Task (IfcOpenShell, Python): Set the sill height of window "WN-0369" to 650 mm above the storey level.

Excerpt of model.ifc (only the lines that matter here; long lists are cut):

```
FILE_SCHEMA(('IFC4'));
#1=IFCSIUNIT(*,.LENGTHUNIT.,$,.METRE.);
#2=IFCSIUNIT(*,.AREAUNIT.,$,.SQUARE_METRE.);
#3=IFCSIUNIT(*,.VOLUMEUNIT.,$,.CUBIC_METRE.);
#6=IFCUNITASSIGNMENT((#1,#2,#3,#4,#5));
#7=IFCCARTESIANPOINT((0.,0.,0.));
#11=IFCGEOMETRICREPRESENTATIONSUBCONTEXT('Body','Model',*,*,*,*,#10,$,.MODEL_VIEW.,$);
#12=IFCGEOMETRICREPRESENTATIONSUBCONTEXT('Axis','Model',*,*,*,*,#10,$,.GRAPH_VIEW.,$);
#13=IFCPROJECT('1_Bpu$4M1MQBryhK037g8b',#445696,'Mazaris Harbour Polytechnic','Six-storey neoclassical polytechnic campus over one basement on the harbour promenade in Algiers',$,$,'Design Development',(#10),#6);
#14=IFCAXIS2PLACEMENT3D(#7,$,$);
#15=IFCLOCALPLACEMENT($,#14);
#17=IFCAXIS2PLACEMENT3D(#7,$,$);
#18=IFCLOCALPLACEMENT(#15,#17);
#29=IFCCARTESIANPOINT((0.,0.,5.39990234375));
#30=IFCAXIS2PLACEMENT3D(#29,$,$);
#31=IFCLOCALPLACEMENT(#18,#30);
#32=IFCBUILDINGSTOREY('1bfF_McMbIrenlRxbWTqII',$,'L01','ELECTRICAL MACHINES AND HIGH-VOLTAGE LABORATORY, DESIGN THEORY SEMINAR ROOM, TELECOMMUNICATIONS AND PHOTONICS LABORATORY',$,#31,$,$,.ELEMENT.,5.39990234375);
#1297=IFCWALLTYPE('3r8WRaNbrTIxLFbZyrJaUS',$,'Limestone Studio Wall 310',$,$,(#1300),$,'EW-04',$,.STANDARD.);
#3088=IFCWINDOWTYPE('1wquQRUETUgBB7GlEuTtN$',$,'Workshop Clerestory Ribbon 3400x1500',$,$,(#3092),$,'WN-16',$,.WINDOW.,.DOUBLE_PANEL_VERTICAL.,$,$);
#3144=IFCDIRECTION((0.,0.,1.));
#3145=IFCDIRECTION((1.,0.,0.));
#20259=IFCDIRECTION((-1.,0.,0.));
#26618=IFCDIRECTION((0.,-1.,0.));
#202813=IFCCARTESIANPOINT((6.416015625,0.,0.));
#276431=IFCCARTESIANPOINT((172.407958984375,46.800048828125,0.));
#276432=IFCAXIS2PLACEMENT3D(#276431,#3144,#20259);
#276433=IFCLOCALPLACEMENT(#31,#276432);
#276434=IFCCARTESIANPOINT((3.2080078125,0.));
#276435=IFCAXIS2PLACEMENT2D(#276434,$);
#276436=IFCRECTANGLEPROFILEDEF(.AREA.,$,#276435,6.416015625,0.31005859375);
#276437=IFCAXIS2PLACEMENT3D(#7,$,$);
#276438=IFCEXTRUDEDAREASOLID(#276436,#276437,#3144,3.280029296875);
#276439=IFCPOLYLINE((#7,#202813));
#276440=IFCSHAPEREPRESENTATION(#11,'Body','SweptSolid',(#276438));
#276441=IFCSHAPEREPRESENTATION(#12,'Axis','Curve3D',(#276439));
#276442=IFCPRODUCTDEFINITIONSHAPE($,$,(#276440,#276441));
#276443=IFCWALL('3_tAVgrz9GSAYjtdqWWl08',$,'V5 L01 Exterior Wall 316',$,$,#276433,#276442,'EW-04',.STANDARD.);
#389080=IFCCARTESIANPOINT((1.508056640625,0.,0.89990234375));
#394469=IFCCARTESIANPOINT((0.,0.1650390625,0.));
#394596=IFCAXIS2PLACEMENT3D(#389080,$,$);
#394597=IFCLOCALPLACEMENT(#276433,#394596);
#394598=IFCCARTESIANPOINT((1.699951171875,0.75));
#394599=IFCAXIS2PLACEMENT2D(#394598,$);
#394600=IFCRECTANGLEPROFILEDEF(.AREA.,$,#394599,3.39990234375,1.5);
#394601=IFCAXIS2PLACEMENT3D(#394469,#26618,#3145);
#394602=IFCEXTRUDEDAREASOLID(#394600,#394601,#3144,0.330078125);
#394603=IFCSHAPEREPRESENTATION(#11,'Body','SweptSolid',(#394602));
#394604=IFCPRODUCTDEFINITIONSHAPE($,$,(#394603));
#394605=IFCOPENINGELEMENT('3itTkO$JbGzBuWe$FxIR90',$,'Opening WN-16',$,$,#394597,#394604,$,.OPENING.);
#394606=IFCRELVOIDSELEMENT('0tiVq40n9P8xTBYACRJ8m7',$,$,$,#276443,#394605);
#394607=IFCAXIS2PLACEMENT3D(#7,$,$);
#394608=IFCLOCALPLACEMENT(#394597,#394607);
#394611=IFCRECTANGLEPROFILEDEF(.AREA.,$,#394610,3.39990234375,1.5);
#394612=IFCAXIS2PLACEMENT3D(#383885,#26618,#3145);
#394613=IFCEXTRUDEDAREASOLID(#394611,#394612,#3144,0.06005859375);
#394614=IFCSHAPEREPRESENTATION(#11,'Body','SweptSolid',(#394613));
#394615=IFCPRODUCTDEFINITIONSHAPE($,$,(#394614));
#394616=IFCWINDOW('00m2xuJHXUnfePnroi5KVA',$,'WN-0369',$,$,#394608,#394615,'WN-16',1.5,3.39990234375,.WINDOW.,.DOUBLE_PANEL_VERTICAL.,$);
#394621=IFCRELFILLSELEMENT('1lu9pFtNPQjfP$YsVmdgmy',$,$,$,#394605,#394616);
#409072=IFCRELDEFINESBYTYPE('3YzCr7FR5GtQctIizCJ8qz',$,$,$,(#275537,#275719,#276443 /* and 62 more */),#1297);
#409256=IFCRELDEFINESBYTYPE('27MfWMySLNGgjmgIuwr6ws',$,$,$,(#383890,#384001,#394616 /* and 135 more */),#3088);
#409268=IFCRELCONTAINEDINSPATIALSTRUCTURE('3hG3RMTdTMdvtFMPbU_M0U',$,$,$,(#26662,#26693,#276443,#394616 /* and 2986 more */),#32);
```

```python
import numpy as np
import ifcopenshell
import ifcopenshell.api.geometry
import ifcopenshell.geom
import ifcopenshell.util.element
import ifcopenshell.util.placement
import ifcopenshell.util.shape
import ifcopenshell.util.unit

model = ifcopenshell.open("model.ifc")
unit_scale = ifcopenshell.util.unit.calculate_unit_scale(model)

window = model.by_id(394616)
opening = window.FillsVoids[0].RelatingOpeningElement
storey = ifcopenshell.util.element.get_container(window, ifc_class="IfcBuildingStorey")
level = ifcopenshell.util.placement.get_local_placement(storey.ObjectPlacement)[2, 3]

# The opening's origin need not be at the sill, so measure its lowest point.
shape = ifcopenshell.geom.create_shape(ifcopenshell.geom.settings(), opening)
bottom = ifcopenshell.util.shape.get_shape_bottom_elevation(shape, shape.geometry) / unit_scale
dz = level + 0.65 / unit_scale - bottom

shift = np.array([0.0, 0.0, dz])
# The window is placed relative to its opening, so it follows when the opening moves.
matrix = ifcopenshell.util.placement.get_local_placement(opening.ObjectPlacement)
matrix[:3, 3] += shift
ifcopenshell.api.geometry.edit_object_placement(
    model, product=opening, matrix=matrix, is_si=False, should_transform_children=True
)

print(f"moved by {dz * unit_scale:+.3f} m")

model.write("model_rev.ifc")
```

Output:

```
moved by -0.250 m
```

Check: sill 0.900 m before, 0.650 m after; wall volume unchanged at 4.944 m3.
